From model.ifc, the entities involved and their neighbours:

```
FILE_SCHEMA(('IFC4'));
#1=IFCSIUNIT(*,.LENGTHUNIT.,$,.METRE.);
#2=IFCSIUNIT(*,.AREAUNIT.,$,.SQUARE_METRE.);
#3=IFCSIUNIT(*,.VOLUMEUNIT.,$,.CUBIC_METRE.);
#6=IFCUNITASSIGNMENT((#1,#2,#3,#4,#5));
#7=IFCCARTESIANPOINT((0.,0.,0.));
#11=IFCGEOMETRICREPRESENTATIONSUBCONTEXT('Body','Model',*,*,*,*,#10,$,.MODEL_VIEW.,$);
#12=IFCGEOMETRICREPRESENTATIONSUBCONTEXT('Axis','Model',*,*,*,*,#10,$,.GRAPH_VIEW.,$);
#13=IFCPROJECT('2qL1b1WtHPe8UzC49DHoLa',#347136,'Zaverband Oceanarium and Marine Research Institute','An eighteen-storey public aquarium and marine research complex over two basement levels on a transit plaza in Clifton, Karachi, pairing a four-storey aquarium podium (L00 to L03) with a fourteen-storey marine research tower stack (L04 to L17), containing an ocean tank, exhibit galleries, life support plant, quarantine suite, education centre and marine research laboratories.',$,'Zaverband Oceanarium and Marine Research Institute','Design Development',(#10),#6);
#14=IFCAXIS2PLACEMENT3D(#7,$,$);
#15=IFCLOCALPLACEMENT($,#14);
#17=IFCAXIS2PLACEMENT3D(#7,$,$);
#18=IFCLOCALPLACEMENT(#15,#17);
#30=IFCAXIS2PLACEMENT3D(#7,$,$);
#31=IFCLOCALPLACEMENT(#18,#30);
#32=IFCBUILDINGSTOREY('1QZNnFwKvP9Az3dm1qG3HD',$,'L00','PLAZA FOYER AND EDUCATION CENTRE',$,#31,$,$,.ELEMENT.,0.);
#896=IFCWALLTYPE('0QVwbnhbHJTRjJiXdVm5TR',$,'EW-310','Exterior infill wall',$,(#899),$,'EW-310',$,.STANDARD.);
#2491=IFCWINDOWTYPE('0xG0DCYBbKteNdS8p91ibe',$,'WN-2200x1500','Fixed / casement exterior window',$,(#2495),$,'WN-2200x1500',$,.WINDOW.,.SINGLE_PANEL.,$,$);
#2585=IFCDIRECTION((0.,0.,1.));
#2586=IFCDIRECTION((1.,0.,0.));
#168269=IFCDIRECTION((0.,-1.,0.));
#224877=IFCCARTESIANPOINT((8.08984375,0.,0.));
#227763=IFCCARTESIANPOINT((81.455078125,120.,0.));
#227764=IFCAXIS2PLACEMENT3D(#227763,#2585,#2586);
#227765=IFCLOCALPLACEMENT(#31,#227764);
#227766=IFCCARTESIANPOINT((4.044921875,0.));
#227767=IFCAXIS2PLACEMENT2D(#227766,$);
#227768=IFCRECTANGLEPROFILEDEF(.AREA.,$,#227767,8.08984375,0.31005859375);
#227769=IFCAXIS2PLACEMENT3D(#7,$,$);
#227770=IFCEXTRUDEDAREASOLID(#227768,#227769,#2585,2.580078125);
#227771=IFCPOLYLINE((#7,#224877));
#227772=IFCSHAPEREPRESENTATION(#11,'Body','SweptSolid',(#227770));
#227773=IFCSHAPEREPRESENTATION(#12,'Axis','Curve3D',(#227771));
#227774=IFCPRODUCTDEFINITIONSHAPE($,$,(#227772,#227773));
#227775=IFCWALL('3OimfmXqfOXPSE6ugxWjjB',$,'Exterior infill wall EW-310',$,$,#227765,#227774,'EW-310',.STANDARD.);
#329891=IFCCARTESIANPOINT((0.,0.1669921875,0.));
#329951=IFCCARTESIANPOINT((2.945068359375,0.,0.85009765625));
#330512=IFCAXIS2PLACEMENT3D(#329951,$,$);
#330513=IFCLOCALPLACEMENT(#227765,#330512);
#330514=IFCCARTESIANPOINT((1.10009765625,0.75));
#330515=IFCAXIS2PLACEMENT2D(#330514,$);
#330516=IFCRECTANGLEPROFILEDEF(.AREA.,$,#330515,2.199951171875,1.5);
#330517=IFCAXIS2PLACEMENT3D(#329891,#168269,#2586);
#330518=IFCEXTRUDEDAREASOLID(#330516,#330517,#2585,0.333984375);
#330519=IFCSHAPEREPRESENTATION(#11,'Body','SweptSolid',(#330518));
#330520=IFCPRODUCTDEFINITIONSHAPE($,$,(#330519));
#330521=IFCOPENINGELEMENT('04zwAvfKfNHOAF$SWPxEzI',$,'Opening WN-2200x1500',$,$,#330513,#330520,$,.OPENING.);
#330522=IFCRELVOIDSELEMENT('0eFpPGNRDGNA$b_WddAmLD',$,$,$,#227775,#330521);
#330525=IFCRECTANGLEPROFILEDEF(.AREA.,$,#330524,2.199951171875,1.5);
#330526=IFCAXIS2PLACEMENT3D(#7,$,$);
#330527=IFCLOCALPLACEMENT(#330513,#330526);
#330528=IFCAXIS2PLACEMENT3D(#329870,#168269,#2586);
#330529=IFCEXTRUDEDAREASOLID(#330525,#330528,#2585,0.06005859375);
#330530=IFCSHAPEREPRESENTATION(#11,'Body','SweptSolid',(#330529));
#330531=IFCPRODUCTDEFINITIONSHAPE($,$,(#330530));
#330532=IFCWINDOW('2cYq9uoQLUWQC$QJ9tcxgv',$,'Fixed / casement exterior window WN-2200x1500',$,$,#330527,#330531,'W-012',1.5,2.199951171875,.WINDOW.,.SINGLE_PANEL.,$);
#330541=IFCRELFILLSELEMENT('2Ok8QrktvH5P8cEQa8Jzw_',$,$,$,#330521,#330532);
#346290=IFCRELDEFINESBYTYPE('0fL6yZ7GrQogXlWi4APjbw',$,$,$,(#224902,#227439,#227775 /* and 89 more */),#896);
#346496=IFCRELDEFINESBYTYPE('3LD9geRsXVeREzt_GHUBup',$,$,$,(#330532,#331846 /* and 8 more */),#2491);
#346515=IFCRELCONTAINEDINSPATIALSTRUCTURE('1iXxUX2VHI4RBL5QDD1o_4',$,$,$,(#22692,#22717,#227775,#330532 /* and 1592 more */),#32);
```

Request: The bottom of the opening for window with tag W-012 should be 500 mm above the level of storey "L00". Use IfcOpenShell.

```python
import numpy as np
import ifcopenshell
import ifcopenshell.api.geometry
import ifcopenshell.geom
import ifcopenshell.util.element
import ifcopenshell.util.placement
import ifcopenshell.util.shape
import ifcopenshell.util.unit

model = ifcopenshell.open("model.ifc")
unit_scale = ifcopenshell.util.unit.calculate_unit_scale(model)

window = model.by_guid("2cYq9uoQLUWQC$QJ9tcxgv")
opening = window.FillsVoids[0].RelatingOpeningElement
storey = ifcopenshell.util.element.get_container(window, ifc_class="IfcBuildingStorey")
level = ifcopenshell.util.placement.get_local_placement(storey.ObjectPlacement)[2, 3]

# The opening's origin need not be at the sill, so measure its lowest point.
shape = ifcopenshell.geom.create_shape(ifcopenshell.geom.settings(), opening)
bottom = ifcopenshell.util.shape.get_shape_bottom_elevation(shape, shape.geometry) / unit_scale
dz = level + 0.5 - bottom

shift = np.array([0.0, 0.0, dz])
# The window is placed relative to its opening, so it follows when the opening moves.
matrix = ifcopenshell.util.placement.get_local_placement(opening.ObjectPlacement)
matrix[:3, 3] += shift
ifcopenshell.api.geometry.edit_object_placement(
    model, product=opening, matrix=matrix, is_si=False, should_transform_children=True
)

print(f"moved by {dz * unit_scale:+.3f} m")

model.write("model_v2.ifc")
```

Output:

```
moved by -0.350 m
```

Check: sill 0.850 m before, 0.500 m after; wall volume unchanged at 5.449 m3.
